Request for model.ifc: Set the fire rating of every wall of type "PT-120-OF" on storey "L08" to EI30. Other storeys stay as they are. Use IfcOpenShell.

First a look at what the model holds.

```python
import ifcopenshell
import ifcopenshell.util.element

model = ifcopenshell.open("model.ifc")
print(model.schema)
storey = next(s for s in model.by_type("IfcBuildingStorey") if s.Name == "L08")
walls = [e for e in ifcopenshell.util.element.get_decomposition(storey) if e.is_a("IfcWall")]
seen = {}
for e in walls:
    element_type = ifcopenshell.util.element.get_type(e)
    key = (element_type.Name if element_type != e and element_type else None, ifcopenshell.util.element.get_pset(e, "Pset_WallCommon", "FireRating"))
    seen[key] = seen.get(key, 0) + 1
for (name, value), count in sorted(seen.items(), key=str):
    print(count, "x", name, "|", value)
```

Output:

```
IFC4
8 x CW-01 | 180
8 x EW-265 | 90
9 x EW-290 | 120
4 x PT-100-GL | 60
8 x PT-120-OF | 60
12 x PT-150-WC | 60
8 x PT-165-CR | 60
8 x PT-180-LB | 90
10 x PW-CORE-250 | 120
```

```python
import ifcopenshell
import ifcopenshell.api.pset
import ifcopenshell.util.element

model = ifcopenshell.open("model.ifc")

storey = next(s for s in model.by_type("IfcBuildingStorey") if s.Name == "L08")
walls = [e for e in ifcopenshell.util.element.get_decomposition(storey) if e.is_a("IfcWall")]

count = 0
for e in walls:
    element_type = ifcopenshell.util.element.get_type(e)
    if element_type in (None, e) or element_type.Name != "PT-120-OF":
        continue
    # add_pset returns the element's existing set when there is one.
    pset = ifcopenshell.api.pset.add_pset(model, product=e, name="Pset_WallCommon")
    ifcopenshell.api.pset.edit_pset(model, pset=pset, properties={"FireRating": "EI30"})
    count += 1

print(count, "walls updated")

model.write("model_v2.ifc")
```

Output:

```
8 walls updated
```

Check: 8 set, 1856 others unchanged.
